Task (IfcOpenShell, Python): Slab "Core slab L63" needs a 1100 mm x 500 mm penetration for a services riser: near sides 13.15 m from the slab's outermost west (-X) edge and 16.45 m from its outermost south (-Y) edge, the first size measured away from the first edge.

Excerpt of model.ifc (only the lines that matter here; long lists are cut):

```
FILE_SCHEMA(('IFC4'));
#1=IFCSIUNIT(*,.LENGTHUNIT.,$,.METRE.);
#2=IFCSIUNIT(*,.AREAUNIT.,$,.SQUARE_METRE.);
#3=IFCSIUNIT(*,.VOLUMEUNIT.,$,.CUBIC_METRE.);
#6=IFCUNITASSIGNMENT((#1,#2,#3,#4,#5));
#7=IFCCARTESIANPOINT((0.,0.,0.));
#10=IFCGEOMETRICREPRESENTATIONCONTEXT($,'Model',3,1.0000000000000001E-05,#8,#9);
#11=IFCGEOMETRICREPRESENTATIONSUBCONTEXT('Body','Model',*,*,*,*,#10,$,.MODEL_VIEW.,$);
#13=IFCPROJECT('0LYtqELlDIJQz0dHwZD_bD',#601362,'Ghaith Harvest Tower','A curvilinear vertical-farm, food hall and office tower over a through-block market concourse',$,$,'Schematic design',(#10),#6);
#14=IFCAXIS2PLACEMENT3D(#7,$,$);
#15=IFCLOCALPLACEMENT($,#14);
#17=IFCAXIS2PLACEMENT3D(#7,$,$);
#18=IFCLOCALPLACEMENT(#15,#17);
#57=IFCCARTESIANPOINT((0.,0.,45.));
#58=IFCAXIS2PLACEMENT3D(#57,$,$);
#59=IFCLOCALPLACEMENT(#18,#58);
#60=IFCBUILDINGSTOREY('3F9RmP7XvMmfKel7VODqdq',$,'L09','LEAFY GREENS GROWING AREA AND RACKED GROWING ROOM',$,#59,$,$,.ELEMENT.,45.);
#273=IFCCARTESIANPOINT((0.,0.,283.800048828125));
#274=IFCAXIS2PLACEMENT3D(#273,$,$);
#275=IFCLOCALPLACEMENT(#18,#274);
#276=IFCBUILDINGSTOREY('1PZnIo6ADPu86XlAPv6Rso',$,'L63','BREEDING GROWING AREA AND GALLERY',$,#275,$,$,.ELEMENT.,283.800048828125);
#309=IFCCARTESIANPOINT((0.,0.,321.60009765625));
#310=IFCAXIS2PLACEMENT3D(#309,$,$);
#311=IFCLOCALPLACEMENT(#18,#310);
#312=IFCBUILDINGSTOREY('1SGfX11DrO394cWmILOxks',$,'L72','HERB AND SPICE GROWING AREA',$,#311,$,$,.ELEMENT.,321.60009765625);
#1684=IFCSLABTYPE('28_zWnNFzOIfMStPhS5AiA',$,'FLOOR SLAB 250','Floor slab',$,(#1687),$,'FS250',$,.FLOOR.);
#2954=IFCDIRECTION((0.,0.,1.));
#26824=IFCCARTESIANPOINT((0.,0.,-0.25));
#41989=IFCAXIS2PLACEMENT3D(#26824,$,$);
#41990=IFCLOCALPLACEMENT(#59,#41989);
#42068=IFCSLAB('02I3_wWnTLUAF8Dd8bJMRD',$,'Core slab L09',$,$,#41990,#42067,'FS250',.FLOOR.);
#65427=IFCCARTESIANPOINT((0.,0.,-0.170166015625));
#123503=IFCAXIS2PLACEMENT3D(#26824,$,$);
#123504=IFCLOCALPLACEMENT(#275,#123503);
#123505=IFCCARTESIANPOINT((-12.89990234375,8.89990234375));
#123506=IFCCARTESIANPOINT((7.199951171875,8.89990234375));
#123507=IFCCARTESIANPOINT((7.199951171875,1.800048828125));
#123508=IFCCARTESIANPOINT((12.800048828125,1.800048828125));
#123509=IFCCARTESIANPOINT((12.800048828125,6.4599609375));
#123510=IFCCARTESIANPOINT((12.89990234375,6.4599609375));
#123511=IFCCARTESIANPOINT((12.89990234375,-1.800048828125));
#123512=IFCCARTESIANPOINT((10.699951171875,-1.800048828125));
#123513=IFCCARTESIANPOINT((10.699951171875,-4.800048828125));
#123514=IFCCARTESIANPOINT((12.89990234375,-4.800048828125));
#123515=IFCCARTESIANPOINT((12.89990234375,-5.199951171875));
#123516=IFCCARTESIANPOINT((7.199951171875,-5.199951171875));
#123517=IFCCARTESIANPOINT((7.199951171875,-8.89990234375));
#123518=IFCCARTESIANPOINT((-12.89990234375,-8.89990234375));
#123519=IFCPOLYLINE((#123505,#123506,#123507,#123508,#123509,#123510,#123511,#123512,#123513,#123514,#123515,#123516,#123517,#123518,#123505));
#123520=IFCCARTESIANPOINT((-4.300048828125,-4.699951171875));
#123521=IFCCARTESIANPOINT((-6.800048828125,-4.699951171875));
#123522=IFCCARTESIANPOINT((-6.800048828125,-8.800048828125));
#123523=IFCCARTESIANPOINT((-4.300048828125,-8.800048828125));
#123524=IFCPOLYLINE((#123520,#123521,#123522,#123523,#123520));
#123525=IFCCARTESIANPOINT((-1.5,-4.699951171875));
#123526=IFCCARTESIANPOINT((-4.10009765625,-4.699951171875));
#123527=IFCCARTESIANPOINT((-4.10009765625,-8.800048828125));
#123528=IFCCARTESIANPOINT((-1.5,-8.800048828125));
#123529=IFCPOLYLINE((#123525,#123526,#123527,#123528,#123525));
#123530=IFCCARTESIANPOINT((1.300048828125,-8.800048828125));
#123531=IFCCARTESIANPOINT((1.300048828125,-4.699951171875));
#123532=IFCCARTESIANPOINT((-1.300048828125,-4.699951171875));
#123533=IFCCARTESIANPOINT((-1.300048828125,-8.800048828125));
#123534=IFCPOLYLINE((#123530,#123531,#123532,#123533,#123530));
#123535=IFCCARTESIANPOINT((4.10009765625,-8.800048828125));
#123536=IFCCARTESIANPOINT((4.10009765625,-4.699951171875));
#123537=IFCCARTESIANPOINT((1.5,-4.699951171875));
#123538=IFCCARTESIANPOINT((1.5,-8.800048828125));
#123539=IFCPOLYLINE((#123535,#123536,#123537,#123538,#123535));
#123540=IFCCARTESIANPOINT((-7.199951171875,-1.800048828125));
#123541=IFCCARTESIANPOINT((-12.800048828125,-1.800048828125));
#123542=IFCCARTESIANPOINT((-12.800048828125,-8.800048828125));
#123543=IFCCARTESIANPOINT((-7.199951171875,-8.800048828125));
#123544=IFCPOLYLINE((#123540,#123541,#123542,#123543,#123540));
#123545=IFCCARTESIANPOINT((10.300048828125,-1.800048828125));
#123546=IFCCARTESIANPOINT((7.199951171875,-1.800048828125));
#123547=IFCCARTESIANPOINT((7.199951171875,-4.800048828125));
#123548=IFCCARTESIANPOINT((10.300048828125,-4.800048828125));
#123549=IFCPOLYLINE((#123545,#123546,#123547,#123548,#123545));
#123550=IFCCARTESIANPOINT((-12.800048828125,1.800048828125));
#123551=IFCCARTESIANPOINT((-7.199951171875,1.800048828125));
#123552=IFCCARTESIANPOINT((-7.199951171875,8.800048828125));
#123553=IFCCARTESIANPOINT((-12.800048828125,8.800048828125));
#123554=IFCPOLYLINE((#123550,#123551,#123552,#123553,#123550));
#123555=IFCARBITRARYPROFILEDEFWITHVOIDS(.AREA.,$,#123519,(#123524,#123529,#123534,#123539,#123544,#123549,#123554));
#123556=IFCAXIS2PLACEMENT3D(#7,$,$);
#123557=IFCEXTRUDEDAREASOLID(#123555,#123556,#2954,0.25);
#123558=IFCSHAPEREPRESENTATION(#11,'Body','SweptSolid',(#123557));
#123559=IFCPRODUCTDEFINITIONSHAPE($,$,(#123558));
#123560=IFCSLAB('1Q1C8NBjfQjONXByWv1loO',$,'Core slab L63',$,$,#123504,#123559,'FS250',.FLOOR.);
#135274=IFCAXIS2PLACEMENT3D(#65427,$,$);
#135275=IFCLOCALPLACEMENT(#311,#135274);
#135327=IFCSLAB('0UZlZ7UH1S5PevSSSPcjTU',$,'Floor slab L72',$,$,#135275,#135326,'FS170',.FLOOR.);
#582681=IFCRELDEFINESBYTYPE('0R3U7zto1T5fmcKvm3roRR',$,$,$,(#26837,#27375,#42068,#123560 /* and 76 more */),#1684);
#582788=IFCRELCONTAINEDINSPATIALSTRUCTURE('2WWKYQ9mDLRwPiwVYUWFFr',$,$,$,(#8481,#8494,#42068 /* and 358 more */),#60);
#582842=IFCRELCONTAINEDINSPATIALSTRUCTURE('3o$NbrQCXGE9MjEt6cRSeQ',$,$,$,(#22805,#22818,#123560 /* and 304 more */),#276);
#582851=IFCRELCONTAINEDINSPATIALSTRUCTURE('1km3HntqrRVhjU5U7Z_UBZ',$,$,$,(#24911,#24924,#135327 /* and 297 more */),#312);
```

```python
import numpy as np
import ifcopenshell
import ifcopenshell.api.feature
import ifcopenshell.api.geometry
import ifcopenshell.api.root
import ifcopenshell.geom
import ifcopenshell.util.placement
import ifcopenshell.util.representation
import ifcopenshell.util.shape
import ifcopenshell.util.unit

model = ifcopenshell.open("model.ifc")
unit_scale = ifcopenshell.util.unit.calculate_unit_scale(model)
settings = ifcopenshell.geom.settings()


def volume(element):
    """Net volume in cubic metres, openings subtracted."""
    shape = ifcopenshell.geom.create_shape(settings, element)
    return ifcopenshell.util.shape.get_volume(shape.geometry)


slab = model.by_id(123560)
before = volume(slab)

# Extent in the slab's own axes, in metres. The edges named are its -X and -Y sides.
slab_shape = ifcopenshell.geom.create_shape(settings, slab)
vertices = ifcopenshell.util.shape.get_vertices(slab_shape.geometry)
x_min, y_min, bottom = vertices.min(axis=0)
top = vertices[:, 2].max()

opening = ifcopenshell.api.root.create_entity(model, ifc_class="IfcOpeningElement", name="Services riser opening", predefined_type="OPENING")
context = ifcopenshell.util.representation.get_context(model, "Model", "Body", "MODEL_VIEW")
width, depth = 1.1, 0.5
outline = [(0.0, 0.0), (width, 0.0), (width, depth), (0.0, depth), (0.0, 0.0)]
# Overshoot both faces by 50 mm so the cut is clean.
shape = ifcopenshell.api.geometry.add_slab_representation(
    model, context=context, depth=top - bottom + 0.1, polyline=outline
)
ifcopenshell.api.geometry.assign_representation(model, product=opening, representation=shape)

matrix = ifcopenshell.util.placement.get_local_placement(slab.ObjectPlacement)
matrix[:, 3] = matrix @ np.append(np.array([x_min + 13.15, y_min + 16.45, bottom - 0.05]) / unit_scale, 1.0)
ifcopenshell.api.geometry.edit_object_placement(model, product=opening, matrix=matrix, is_si=False)
ifcopenshell.api.feature.add_feature(model, feature=opening, element=slab)

after = volume(slab)

print(f"slab volume {before:.3f} -> {after:.3f} m3")

model.write("model-out.ifc")
```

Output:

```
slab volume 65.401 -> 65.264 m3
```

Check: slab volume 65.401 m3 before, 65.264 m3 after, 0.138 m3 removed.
